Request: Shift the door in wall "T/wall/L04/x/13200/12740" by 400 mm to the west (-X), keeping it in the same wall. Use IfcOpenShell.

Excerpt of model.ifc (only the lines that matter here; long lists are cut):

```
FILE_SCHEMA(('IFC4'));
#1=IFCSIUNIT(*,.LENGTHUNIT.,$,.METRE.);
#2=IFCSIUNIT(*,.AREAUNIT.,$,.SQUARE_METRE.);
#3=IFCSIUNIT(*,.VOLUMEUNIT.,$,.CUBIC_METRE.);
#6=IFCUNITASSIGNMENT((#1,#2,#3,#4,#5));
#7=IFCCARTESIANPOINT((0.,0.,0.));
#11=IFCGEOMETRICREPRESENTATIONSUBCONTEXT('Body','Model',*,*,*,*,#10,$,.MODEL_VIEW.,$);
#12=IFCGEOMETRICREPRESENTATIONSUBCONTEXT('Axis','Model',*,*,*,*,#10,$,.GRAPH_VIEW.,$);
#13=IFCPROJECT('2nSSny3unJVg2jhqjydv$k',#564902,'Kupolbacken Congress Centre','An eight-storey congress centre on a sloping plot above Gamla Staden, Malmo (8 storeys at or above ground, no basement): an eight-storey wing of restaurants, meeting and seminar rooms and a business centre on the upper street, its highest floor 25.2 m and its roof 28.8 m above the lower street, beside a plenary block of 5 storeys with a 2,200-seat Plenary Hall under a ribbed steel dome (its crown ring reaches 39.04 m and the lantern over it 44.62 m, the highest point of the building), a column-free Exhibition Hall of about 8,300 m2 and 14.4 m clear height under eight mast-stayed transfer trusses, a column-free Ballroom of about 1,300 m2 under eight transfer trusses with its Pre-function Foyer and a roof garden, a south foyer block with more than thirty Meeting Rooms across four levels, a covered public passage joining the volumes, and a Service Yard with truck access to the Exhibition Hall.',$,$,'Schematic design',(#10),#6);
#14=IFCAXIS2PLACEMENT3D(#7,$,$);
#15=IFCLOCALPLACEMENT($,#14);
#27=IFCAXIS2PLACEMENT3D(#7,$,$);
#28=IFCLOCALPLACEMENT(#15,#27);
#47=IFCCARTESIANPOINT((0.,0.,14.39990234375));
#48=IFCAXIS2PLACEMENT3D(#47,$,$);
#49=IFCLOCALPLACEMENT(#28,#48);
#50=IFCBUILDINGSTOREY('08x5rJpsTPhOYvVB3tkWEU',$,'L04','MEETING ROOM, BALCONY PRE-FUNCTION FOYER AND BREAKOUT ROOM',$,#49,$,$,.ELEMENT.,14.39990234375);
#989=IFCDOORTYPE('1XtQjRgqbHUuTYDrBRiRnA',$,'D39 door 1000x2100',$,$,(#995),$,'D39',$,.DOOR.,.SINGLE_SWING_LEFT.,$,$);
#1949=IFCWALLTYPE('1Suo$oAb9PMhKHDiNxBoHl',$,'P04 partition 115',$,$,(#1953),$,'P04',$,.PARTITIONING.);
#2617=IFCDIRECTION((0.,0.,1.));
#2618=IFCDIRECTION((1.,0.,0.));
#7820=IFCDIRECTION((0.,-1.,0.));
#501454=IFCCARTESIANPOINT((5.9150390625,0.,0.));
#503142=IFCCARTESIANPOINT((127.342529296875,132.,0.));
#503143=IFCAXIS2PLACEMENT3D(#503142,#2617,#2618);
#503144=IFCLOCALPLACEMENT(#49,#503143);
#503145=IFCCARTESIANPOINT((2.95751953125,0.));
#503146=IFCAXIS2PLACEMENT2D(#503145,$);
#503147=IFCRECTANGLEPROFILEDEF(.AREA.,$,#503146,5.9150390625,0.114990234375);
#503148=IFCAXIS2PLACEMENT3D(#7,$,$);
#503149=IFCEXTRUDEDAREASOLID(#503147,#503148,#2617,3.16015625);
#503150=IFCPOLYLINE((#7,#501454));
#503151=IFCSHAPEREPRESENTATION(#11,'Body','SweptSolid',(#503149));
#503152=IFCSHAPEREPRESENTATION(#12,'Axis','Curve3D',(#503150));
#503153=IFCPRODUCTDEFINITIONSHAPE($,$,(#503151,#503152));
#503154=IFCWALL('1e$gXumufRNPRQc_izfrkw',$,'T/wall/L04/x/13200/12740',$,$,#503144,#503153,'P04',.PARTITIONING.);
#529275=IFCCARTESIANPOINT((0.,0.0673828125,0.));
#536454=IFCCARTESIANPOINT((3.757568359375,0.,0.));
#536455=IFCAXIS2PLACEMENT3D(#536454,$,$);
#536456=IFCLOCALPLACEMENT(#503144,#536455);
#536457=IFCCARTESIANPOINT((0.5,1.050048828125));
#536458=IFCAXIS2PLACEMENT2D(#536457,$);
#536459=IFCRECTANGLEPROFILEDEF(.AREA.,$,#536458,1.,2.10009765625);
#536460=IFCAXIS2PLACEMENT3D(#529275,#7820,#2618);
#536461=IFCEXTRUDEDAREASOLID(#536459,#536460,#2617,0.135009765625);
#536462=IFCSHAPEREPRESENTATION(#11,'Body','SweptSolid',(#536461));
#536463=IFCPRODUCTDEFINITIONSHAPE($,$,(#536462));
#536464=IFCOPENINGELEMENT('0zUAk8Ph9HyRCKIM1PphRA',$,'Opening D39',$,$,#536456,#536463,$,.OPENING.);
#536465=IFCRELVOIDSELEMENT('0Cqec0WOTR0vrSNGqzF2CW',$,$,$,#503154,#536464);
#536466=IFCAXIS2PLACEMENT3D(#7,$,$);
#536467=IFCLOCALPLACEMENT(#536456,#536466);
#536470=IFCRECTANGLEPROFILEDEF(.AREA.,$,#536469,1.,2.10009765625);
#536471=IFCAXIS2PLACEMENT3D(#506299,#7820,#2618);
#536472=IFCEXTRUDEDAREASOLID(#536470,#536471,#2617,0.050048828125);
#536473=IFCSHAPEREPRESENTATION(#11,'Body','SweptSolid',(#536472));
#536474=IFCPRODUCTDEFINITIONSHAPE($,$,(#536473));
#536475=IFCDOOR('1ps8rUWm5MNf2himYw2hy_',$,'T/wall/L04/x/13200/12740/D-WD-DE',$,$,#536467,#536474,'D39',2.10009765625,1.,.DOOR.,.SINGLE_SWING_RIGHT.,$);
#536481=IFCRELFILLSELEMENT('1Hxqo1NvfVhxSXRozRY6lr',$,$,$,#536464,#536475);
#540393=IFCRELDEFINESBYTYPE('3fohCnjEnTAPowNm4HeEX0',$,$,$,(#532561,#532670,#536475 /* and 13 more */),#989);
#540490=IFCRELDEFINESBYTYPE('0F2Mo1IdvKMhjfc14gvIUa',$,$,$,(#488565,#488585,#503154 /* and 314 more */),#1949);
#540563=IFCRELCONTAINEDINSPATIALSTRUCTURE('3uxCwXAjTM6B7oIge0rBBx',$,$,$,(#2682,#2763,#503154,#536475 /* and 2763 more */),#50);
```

```python
import ifcopenshell
import ifcopenshell.api.geometry
import ifcopenshell.util.placement
import ifcopenshell.util.unit

model = ifcopenshell.open("model.ifc")
unit_scale = ifcopenshell.util.unit.calculate_unit_scale(model)

door = model.by_guid("1ps8rUWm5MNf2himYw2hy_")
opening = door.FillsVoids[0].RelatingOpeningElement
wall = opening.VoidsElements[0].RelatingBuildingElement

wall_matrix = ifcopenshell.util.placement.get_local_placement(wall.ObjectPlacement)
shift = wall_matrix[:3, 0] * -0.4 / unit_scale
before = ifcopenshell.util.placement.get_local_placement(door.ObjectPlacement)[:3, 3].copy()

# The door is placed relative to its opening, so it follows when the opening moves.
matrix = ifcopenshell.util.placement.get_local_placement(opening.ObjectPlacement)
matrix[:3, 3] += shift
ifcopenshell.api.geometry.edit_object_placement(
    model, product=opening, matrix=matrix, is_si=False, should_transform_children=True
)

after = ifcopenshell.util.placement.get_local_placement(door.ObjectPlacement)[:3, 3]
print("door moved by", (after - before).round(3) + 0.0)

model.write("model_v2.ifc")
```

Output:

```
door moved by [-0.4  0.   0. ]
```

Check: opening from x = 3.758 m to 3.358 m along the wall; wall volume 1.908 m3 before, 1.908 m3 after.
